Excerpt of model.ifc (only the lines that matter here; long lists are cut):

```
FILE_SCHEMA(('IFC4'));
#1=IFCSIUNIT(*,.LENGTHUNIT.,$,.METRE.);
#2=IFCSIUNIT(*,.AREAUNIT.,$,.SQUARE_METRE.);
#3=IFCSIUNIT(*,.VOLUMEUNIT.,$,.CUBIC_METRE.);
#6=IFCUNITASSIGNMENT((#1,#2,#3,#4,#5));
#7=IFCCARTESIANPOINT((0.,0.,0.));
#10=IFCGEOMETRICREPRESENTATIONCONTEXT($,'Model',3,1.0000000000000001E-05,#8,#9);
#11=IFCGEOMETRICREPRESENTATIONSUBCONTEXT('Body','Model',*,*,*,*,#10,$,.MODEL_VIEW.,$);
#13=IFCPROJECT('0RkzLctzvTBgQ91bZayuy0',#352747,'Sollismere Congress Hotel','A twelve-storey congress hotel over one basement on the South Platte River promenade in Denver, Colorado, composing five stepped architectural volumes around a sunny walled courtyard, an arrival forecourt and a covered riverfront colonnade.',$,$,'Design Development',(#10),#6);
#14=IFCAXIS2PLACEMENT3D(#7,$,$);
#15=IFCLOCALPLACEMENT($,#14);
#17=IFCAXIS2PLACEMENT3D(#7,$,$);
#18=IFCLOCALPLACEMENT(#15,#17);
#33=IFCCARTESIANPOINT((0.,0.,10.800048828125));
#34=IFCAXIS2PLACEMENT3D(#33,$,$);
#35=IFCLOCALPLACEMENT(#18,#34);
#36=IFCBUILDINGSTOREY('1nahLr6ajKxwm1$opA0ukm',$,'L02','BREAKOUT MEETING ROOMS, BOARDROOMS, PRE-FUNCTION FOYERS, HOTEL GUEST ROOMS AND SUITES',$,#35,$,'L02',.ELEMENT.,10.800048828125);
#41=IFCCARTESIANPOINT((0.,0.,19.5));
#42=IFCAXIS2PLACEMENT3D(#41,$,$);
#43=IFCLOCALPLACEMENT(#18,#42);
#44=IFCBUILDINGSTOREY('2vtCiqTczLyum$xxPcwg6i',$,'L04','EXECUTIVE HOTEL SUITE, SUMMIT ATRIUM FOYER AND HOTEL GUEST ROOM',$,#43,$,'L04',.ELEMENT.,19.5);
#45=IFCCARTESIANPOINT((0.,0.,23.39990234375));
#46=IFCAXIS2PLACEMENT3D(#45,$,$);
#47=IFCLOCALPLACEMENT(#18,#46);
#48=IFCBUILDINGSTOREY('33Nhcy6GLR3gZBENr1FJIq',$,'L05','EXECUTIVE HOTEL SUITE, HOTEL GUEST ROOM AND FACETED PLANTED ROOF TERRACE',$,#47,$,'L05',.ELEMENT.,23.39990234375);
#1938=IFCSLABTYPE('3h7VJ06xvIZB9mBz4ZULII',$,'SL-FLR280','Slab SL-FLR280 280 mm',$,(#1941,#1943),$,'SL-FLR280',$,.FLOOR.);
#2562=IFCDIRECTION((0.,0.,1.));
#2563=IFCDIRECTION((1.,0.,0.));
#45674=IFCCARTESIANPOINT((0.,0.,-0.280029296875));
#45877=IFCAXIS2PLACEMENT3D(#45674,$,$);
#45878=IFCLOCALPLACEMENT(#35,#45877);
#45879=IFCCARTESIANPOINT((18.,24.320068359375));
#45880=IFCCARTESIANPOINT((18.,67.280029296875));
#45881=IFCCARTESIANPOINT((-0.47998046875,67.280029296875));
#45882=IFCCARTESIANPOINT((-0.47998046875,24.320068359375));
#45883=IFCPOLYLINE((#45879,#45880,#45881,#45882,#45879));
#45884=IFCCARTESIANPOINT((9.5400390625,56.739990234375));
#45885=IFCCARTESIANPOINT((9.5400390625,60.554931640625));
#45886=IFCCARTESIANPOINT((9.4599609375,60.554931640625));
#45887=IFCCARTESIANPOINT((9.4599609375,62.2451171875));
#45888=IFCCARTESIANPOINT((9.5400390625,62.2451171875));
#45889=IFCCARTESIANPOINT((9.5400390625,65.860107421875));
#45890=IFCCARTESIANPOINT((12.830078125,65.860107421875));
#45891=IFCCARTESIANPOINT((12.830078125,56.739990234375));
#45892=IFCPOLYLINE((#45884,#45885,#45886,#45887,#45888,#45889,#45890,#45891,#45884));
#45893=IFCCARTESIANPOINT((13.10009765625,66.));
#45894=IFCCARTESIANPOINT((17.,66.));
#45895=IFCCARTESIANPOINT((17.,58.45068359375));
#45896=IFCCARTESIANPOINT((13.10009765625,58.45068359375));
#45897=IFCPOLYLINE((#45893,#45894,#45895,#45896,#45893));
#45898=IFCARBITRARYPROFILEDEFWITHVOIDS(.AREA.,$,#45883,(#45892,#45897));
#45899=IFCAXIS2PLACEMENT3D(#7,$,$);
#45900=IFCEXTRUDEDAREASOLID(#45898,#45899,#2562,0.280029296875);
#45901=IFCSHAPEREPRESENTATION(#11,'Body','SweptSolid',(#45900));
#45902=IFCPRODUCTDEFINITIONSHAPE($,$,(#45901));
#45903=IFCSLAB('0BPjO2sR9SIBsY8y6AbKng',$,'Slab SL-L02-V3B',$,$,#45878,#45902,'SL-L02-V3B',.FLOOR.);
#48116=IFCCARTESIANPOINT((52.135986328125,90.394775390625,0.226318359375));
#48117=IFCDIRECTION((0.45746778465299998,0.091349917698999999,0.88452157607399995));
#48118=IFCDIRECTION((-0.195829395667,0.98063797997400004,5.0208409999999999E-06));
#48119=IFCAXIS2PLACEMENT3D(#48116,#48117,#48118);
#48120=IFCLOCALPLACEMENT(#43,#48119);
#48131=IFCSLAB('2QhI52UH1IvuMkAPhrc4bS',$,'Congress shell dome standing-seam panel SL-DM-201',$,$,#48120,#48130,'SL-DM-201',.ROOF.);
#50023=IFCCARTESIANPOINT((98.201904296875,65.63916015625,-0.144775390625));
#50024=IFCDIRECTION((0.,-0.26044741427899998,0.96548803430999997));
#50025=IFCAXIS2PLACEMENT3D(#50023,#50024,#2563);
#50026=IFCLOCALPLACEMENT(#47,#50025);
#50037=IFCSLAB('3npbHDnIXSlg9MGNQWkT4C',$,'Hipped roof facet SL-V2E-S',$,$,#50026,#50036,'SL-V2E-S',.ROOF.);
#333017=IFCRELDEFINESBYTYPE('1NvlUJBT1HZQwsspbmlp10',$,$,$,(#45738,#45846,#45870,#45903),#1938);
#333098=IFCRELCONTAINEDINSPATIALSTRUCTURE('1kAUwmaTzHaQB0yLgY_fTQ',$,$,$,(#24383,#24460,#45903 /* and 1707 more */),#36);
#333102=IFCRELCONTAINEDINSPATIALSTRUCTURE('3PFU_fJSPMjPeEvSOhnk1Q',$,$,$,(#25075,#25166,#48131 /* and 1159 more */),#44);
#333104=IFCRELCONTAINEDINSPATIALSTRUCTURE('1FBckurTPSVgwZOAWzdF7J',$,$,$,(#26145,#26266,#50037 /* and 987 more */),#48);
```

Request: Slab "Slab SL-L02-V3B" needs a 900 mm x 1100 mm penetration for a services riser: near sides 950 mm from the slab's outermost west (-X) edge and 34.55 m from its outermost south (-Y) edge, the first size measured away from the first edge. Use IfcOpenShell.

```python
import numpy as np
import ifcopenshell
import ifcopenshell.api.feature
import ifcopenshell.api.geometry
import ifcopenshell.api.root
import ifcopenshell.geom
import ifcopenshell.util.placement
import ifcopenshell.util.representation
import ifcopenshell.util.shape
import ifcopenshell.util.unit

model = ifcopenshell.open("model.ifc")
unit_scale = ifcopenshell.util.unit.calculate_unit_scale(model)
settings = ifcopenshell.geom.settings()


def volume(element):
    """Net volume in cubic metres, openings subtracted."""
    shape = ifcopenshell.geom.create_shape(settings, element)
    return ifcopenshell.util.shape.get_volume(shape.geometry)


slab = model.by_guid("0BPjO2sR9SIBsY8y6AbKng")
before = volume(slab)

# Extent in the slab's own axes, in metres. The edges named are its -X and -Y sides.
slab_shape = ifcopenshell.geom.create_shape(settings, slab)
vertices = ifcopenshell.util.shape.get_vertices(slab_shape.geometry)
x_min, y_min, bottom = vertices.min(axis=0)
top = vertices[:, 2].max()

opening = ifcopenshell.api.root.create_entity(model, ifc_class="IfcOpeningElement", name="Services riser opening", predefined_type="OPENING")
context = ifcopenshell.util.representation.get_context(model, "Model", "Body", "MODEL_VIEW")
width, depth = 0.9, 1.1
outline = [(0.0, 0.0), (width, 0.0), (width, depth), (0.0, depth), (0.0, 0.0)]
# Overshoot both faces by 50 mm so the cut is clean.
shape = ifcopenshell.api.geometry.add_slab_representation(
    model, context=context, depth=top - bottom + 0.1, polyline=outline
)
ifcopenshell.api.geometry.assign_representation(model, product=opening, representation=shape)

matrix = ifcopenshell.util.placement.get_local_placement(slab.ObjectPlacement)
matrix[:, 3] = matrix @ np.append(np.array([x_min + 0.95, y_min + 34.55, bottom - 0.05]) / unit_scale, 1.0)
ifcopenshell.api.geometry.edit_object_placement(model, product=opening, matrix=matrix, is_si=False)
ifcopenshell.api.feature.add_feature(model, feature=opening, element=slab)

after = volume(slab)

print(f"slab volume {before:.3f} -> {after:.3f} m3")

model.write("model_v2.ifc")
```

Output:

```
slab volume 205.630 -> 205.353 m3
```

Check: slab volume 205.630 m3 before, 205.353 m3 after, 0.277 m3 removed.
